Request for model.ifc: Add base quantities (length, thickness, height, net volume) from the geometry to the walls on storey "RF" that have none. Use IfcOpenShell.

First a look at what the model holds.

```python
import ifcopenshell
import ifcopenshell.util.element
import ifcopenshell.util.unit

model = ifcopenshell.open("model.ifc")
print(model.schema)
for unit_type in ("LENGTHUNIT", "AREAUNIT", "VOLUMEUNIT"):
    print(unit_type, ifcopenshell.util.unit.calculate_unit_scale(model, unit_type))
storey = next(s for s in model.by_type("IfcBuildingStorey") if s.Name == "RF")
walls = [e for e in ifcopenshell.util.element.get_decomposition(storey) if e.is_a("IfcWall")]
for e in sorted(walls, key=lambda e: e.id()):
    print(e.id(), e.is_a(), e.Name, list(ifcopenshell.util.element.get_psets(e, qtos_only=True)), sep=" | ")
```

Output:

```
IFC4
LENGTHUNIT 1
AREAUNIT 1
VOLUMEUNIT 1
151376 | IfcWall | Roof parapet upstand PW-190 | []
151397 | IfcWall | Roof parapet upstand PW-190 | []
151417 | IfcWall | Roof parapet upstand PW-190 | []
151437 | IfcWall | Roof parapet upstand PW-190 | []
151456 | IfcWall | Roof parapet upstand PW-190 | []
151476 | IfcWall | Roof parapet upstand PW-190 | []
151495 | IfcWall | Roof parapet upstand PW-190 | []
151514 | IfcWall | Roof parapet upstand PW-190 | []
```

```python
import ifcopenshell
import ifcopenshell.api.pset
import ifcopenshell.geom
import ifcopenshell.util.element
import ifcopenshell.util.shape
import ifcopenshell.util.unit

model = ifcopenshell.open("model.ifc")
unit_scale = ifcopenshell.util.unit.calculate_unit_scale(model)
volume_scale = ifcopenshell.util.unit.calculate_unit_scale(model, "VOLUMEUNIT")
settings = ifcopenshell.geom.settings()

storey = next(s for s in model.by_type("IfcBuildingStorey") if s.Name == "RF")
walls = [e for e in ifcopenshell.util.element.get_decomposition(storey) if e.is_a("IfcWall")]

for e in sorted(walls, key=lambda e: e.id()):
    if ifcopenshell.util.element.get_psets(e, qtos_only=True, should_inherit=False):
        continue
    # Geometry comes back in metres, in the element's own axes.
    shape = ifcopenshell.geom.create_shape(settings, e)
    values = {
        "Length": ifcopenshell.util.shape.get_x(shape.geometry) / unit_scale,
        "Width": ifcopenshell.util.shape.get_y(shape.geometry) / unit_scale,
        "Height": ifcopenshell.util.shape.get_z(shape.geometry) / unit_scale,
        "NetVolume": ifcopenshell.util.shape.get_volume(shape.geometry) / volume_scale,
    }
    qto = ifcopenshell.api.pset.add_qto(model, product=e, name="Qto_WallBaseQuantities")
    ifcopenshell.api.pset.edit_qto(model, qto=qto, properties=values)
    print(e.id(), {k: round(v, 3) for k, v in values.items()})

model.write("model_v2.ifc")
```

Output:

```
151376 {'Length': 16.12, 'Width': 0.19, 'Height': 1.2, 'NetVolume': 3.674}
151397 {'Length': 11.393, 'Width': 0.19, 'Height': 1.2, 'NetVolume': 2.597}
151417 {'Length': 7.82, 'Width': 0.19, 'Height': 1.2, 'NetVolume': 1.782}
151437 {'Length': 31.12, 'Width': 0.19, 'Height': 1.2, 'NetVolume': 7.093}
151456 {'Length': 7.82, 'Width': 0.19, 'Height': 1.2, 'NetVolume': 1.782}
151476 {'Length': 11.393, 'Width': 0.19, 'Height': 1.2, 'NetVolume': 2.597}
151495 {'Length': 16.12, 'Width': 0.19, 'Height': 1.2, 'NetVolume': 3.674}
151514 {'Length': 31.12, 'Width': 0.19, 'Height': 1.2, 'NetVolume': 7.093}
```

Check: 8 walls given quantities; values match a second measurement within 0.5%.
